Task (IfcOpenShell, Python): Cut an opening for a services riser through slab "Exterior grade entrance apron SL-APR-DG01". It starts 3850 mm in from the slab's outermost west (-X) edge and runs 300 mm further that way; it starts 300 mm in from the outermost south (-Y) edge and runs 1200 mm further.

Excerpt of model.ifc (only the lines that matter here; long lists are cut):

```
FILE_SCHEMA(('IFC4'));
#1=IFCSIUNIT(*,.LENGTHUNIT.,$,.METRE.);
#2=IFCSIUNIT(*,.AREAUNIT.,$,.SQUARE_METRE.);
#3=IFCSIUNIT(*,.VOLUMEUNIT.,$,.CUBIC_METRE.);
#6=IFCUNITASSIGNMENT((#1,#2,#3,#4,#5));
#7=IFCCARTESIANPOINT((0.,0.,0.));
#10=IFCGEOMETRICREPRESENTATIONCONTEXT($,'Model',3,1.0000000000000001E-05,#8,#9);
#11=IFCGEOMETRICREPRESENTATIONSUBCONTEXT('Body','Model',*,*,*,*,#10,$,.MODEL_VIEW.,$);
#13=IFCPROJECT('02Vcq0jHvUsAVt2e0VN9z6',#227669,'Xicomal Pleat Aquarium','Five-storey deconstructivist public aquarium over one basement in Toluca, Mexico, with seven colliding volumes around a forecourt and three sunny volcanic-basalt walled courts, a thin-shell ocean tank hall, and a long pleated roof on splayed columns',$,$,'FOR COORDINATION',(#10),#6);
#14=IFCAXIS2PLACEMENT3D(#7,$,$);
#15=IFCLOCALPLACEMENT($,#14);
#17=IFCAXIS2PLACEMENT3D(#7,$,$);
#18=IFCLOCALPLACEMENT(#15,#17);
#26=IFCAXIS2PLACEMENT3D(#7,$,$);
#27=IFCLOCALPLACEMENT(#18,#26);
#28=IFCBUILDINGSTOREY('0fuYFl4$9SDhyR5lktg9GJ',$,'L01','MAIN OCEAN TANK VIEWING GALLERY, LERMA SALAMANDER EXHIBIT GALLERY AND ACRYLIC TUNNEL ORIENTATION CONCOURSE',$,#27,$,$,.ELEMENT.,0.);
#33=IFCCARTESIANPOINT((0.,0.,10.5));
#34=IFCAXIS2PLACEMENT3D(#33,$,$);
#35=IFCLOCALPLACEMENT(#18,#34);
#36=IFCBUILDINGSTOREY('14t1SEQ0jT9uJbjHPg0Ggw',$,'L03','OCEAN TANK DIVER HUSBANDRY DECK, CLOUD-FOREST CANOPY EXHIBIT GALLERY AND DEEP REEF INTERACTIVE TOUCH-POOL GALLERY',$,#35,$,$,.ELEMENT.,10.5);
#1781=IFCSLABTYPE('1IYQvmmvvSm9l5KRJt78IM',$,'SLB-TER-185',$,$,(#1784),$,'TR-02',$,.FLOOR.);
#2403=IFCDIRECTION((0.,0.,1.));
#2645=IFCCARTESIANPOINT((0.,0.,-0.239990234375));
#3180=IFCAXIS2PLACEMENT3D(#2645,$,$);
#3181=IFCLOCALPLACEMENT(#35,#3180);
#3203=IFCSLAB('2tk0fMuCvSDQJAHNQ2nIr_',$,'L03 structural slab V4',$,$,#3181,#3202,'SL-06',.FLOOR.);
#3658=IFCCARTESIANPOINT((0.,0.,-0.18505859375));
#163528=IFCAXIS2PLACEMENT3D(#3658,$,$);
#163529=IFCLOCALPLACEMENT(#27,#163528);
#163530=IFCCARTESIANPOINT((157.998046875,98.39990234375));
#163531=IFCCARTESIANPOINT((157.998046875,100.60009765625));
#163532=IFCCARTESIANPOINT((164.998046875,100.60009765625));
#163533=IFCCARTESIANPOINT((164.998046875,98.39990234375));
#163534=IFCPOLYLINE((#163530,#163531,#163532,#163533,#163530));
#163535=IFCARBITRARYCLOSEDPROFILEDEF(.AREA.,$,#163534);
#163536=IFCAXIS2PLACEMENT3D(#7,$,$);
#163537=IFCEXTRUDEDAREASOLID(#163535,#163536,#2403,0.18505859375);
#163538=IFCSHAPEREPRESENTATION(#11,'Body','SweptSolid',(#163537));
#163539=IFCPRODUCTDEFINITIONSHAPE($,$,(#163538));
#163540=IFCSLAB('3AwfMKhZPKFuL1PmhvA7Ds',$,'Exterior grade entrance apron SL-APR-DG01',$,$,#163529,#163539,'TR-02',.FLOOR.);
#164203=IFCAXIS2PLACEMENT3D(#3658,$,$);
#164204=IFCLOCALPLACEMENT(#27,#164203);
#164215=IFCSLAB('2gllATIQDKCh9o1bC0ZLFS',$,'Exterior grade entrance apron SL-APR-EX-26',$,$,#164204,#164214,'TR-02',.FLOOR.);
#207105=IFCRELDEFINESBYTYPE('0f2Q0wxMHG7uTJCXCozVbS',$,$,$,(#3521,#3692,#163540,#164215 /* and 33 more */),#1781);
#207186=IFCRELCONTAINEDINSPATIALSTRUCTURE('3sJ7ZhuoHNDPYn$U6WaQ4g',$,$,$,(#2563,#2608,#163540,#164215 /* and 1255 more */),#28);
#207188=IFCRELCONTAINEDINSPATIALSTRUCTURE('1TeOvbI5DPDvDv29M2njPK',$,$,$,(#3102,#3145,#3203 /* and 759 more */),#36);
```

```python
import numpy as np
import ifcopenshell
import ifcopenshell.api.feature
import ifcopenshell.api.geometry
import ifcopenshell.api.root
import ifcopenshell.geom
import ifcopenshell.util.placement
import ifcopenshell.util.representation
import ifcopenshell.util.shape
import ifcopenshell.util.unit

model = ifcopenshell.open("model.ifc")
unit_scale = ifcopenshell.util.unit.calculate_unit_scale(model)
settings = ifcopenshell.geom.settings()


def volume(element):
    """Net volume in cubic metres, openings subtracted."""
    shape = ifcopenshell.geom.create_shape(settings, element)
    return ifcopenshell.util.shape.get_volume(shape.geometry)


slab = model.by_guid("3AwfMKhZPKFuL1PmhvA7Ds")
before = volume(slab)

# Extent in the slab's own axes, in metres. The edges named are its -X and -Y sides.
slab_shape = ifcopenshell.geom.create_shape(settings, slab)
vertices = ifcopenshell.util.shape.get_vertices(slab_shape.geometry)
x_min, y_min, bottom = vertices.min(axis=0)
top = vertices[:, 2].max()

opening = ifcopenshell.api.root.create_entity(model, ifc_class="IfcOpeningElement", name="Services riser opening", predefined_type="OPENING")
context = ifcopenshell.util.representation.get_context(model, "Model", "Body", "MODEL_VIEW")
width, depth = 0.3, 1.2
outline = [(0.0, 0.0), (width, 0.0), (width, depth), (0.0, depth), (0.0, 0.0)]
# Overshoot both faces by 50 mm so the cut is clean.
shape = ifcopenshell.api.geometry.add_slab_representation(
    model, context=context, depth=top - bottom + 0.1, polyline=outline
)
ifcopenshell.api.geometry.assign_representation(model, product=opening, representation=shape)

matrix = ifcopenshell.util.placement.get_local_placement(slab.ObjectPlacement)
matrix[:, 3] = matrix @ np.append(np.array([x_min + 3.85, y_min + 0.3, bottom - 0.05]) / unit_scale, 1.0)
ifcopenshell.api.geometry.edit_object_placement(model, product=opening, matrix=matrix, is_si=False)
ifcopenshell.api.feature.add_feature(model, feature=opening, element=slab)

after = volume(slab)

print(f"slab volume {before:.3f} -> {after:.3f} m3")

model.write("model_rev.ifc")
```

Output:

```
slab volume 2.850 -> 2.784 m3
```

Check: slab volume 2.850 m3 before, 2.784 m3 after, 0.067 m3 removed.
